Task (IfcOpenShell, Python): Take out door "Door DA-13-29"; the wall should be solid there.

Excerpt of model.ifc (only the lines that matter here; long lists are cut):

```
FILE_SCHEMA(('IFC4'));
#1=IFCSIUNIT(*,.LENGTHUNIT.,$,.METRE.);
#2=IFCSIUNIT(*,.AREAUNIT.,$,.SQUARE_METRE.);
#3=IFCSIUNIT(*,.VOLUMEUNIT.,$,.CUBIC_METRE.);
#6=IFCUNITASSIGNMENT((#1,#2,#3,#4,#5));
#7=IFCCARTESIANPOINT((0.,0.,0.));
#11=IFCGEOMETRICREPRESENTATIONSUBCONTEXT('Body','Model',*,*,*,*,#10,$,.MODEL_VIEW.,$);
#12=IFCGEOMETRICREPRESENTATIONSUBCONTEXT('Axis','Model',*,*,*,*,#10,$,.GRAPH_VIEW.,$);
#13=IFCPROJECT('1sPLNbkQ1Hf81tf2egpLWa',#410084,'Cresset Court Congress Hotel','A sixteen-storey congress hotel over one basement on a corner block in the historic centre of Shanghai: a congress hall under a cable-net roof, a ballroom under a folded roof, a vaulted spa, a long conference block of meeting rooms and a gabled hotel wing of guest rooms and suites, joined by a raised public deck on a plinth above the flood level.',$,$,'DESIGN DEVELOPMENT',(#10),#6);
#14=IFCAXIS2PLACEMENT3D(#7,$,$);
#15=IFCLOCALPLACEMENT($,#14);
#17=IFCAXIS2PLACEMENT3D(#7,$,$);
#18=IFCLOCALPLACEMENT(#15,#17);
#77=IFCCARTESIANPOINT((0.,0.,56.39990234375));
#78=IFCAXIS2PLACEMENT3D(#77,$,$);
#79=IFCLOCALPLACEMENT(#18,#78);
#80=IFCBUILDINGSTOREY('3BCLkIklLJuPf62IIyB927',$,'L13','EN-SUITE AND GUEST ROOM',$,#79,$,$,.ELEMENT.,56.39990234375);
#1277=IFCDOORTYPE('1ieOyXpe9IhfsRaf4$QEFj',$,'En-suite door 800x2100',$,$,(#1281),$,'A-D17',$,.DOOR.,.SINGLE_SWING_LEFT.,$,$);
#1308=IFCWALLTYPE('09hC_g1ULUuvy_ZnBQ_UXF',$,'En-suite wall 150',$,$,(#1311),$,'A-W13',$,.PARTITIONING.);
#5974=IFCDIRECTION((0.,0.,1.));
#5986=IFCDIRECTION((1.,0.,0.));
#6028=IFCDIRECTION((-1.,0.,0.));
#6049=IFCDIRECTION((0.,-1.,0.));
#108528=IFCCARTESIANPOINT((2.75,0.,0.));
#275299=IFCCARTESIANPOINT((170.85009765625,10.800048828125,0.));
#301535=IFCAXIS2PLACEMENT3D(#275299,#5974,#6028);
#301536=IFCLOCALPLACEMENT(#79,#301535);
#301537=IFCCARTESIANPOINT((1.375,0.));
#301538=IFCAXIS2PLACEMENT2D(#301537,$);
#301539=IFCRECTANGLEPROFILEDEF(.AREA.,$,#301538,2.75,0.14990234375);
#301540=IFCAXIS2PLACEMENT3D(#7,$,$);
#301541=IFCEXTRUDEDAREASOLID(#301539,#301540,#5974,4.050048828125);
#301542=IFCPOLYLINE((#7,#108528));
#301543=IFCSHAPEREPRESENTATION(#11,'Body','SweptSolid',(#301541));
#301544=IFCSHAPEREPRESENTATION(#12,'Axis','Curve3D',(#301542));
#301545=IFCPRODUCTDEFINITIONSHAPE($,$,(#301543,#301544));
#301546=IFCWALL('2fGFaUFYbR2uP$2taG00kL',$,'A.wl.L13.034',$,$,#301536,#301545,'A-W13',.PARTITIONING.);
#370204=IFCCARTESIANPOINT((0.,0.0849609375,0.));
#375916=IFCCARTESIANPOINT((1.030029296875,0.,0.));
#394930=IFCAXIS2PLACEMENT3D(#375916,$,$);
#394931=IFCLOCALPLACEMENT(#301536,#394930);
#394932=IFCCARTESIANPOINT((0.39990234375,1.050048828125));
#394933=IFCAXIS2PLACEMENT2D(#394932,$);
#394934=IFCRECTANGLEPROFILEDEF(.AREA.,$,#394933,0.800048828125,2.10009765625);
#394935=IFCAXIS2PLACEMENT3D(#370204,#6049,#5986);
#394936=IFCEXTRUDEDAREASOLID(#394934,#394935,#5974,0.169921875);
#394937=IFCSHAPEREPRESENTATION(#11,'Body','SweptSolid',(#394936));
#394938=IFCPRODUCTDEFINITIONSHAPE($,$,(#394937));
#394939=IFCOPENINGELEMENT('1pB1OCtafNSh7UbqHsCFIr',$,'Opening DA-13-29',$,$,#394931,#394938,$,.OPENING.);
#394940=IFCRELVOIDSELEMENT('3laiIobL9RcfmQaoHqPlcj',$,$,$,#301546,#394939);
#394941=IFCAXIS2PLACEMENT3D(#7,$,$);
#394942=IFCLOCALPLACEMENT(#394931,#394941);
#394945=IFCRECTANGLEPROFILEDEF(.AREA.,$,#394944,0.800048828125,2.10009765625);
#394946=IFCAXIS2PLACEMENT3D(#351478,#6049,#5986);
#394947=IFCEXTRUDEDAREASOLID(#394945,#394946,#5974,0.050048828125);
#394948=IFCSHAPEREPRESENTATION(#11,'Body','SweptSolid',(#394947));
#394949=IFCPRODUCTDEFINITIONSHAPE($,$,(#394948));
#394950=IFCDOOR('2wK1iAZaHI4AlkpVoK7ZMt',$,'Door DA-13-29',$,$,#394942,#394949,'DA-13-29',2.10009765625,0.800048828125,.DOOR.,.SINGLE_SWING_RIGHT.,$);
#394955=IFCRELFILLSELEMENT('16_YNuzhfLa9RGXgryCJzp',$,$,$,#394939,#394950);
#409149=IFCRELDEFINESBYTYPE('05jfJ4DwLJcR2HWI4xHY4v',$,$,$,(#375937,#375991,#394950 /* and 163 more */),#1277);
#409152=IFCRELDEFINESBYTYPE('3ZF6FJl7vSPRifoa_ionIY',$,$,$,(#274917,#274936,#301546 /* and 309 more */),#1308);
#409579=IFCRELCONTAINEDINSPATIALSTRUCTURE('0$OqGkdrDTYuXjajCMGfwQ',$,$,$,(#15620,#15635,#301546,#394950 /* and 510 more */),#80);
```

```python
import ifcopenshell
import ifcopenshell.api.feature
import ifcopenshell.api.root
import ifcopenshell.geom
import ifcopenshell.util.shape

model = ifcopenshell.open("model.ifc")
settings = ifcopenshell.geom.settings()


def volume(element):
    """Net volume in cubic metres, openings subtracted."""
    shape = ifcopenshell.geom.create_shape(settings, element)
    return ifcopenshell.util.shape.get_volume(shape.geometry)


door = model.by_id(394950)
opening = door.FillsVoids[0].RelatingOpeningElement
wall = opening.VoidsElements[0].RelatingBuildingElement
before = volume(wall)

ifcopenshell.api.root.remove_product(model, product=door)
ifcopenshell.api.feature.remove_feature(model, feature=opening)

after = volume(wall)

print(f"wall volume {before:.3f} -> {after:.3f} m3")

model.write("model_updated.ifc")
```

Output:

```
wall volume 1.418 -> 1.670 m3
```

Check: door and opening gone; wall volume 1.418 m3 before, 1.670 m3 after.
